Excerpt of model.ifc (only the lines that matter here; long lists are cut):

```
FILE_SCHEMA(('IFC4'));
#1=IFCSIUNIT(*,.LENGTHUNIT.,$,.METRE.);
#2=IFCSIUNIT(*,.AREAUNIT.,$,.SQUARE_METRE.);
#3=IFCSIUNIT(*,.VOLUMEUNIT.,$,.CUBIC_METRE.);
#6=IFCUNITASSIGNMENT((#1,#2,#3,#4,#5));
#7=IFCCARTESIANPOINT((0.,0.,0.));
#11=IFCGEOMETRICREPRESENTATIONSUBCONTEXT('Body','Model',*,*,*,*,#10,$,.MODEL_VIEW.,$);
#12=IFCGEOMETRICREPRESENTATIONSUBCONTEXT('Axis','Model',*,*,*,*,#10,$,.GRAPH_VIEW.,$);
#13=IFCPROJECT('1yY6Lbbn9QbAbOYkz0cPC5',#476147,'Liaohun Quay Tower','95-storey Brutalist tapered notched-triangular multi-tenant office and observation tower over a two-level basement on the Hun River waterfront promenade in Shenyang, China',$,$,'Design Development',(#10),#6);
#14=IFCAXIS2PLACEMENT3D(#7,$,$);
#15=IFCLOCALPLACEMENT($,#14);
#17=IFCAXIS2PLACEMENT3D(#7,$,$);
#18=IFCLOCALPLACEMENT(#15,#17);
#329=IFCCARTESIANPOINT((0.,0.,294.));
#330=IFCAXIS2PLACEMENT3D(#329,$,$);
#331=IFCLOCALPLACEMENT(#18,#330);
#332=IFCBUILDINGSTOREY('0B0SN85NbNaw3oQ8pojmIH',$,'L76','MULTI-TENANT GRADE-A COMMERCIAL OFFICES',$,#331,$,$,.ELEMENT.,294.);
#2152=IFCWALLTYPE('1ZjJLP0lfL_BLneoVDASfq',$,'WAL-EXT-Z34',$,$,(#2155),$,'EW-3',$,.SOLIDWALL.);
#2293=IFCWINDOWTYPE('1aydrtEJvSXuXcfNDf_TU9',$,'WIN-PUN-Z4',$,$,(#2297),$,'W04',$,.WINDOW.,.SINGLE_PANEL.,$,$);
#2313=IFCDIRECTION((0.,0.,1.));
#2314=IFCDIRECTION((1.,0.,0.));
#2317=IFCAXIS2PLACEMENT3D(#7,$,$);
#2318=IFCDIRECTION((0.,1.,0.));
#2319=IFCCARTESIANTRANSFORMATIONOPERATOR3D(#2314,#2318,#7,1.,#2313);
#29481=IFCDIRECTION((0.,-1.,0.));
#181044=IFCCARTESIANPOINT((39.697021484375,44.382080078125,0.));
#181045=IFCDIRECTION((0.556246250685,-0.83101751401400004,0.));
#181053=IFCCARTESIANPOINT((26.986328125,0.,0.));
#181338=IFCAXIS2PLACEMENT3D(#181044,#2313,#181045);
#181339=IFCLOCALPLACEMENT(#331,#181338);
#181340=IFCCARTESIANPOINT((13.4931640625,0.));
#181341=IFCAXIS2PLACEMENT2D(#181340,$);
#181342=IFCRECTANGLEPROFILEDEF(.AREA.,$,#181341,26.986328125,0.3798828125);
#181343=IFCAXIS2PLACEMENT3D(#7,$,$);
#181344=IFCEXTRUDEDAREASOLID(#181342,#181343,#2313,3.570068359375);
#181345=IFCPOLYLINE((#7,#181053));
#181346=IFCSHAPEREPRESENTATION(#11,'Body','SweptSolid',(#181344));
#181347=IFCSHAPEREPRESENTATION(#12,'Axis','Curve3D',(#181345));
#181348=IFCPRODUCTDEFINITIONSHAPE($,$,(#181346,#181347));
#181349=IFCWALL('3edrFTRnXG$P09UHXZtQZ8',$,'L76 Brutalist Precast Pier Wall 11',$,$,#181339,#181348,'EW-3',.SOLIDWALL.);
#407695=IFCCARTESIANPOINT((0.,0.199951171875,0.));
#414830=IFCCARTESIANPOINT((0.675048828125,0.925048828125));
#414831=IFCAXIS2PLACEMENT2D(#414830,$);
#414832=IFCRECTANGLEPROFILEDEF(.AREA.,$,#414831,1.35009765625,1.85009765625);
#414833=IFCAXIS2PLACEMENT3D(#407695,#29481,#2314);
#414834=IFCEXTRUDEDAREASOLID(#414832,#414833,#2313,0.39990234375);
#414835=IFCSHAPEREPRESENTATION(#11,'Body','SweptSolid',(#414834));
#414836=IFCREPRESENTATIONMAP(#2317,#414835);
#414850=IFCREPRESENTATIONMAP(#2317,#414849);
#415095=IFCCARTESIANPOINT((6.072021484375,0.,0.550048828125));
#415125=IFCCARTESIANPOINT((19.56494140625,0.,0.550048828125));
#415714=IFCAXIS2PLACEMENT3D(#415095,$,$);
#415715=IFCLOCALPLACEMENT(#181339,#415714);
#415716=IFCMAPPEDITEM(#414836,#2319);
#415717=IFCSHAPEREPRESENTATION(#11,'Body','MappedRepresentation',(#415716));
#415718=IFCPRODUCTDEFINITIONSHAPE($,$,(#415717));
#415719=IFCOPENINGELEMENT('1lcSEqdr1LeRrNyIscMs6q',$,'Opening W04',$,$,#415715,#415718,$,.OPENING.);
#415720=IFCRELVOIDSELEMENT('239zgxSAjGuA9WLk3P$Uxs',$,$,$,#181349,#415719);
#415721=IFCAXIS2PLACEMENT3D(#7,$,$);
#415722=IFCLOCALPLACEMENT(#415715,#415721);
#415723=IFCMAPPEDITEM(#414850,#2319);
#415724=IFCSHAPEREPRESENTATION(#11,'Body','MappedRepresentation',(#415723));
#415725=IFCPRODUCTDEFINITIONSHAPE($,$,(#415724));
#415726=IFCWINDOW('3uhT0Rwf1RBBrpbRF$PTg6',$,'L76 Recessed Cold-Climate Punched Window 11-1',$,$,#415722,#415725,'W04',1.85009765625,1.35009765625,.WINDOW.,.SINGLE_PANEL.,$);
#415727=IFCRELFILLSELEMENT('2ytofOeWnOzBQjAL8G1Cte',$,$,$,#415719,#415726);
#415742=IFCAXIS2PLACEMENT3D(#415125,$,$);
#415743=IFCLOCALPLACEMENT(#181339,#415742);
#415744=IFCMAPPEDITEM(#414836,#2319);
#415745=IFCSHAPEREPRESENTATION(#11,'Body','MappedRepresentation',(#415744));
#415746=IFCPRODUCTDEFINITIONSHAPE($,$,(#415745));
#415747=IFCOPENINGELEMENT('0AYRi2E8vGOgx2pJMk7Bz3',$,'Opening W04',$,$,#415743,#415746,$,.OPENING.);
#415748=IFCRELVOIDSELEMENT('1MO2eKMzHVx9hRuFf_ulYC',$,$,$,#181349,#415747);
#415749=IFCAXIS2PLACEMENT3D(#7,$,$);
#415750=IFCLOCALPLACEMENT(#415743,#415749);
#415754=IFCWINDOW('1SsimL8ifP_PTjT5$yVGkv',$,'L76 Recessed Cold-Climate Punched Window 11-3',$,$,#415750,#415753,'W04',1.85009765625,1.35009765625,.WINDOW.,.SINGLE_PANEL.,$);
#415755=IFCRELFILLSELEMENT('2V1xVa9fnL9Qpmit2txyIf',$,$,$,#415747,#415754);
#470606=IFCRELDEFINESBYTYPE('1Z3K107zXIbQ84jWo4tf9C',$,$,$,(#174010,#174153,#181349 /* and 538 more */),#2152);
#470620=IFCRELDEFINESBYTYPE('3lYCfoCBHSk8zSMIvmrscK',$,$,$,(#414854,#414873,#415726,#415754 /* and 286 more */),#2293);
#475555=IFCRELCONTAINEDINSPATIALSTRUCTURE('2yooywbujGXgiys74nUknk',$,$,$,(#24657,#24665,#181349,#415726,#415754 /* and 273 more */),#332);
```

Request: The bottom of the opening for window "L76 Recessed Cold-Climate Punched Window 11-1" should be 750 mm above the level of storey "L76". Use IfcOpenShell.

```python
import numpy as np
import ifcopenshell
import ifcopenshell.api.geometry
import ifcopenshell.geom
import ifcopenshell.util.element
import ifcopenshell.util.placement
import ifcopenshell.util.shape
import ifcopenshell.util.unit

model = ifcopenshell.open("model.ifc")
unit_scale = ifcopenshell.util.unit.calculate_unit_scale(model)

window = model.by_guid("3uhT0Rwf1RBBrpbRF$PTg6")
opening = window.FillsVoids[0].RelatingOpeningElement
storey = ifcopenshell.util.element.get_container(window, ifc_class="IfcBuildingStorey")
level = ifcopenshell.util.placement.get_local_placement(storey.ObjectPlacement)[2, 3]

# The opening's origin need not be at the sill, so measure its lowest point.
shape = ifcopenshell.geom.create_shape(ifcopenshell.geom.settings(), opening)
bottom = ifcopenshell.util.shape.get_shape_bottom_elevation(shape, shape.geometry) / unit_scale
dz = level + 0.75 / unit_scale - bottom

shift = np.array([0.0, 0.0, dz])
# The window is placed relative to its opening, so it follows when the opening moves.
matrix = ifcopenshell.util.placement.get_local_placement(opening.ObjectPlacement)
matrix[:3, 3] += shift
ifcopenshell.api.geometry.edit_object_placement(
    model, product=opening, matrix=matrix, is_si=False, should_transform_children=True
)

print(f"moved by {dz * unit_scale:+.3f} m")

model.write("model_v2.ifc")
```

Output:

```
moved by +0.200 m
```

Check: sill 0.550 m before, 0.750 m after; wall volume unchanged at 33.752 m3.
